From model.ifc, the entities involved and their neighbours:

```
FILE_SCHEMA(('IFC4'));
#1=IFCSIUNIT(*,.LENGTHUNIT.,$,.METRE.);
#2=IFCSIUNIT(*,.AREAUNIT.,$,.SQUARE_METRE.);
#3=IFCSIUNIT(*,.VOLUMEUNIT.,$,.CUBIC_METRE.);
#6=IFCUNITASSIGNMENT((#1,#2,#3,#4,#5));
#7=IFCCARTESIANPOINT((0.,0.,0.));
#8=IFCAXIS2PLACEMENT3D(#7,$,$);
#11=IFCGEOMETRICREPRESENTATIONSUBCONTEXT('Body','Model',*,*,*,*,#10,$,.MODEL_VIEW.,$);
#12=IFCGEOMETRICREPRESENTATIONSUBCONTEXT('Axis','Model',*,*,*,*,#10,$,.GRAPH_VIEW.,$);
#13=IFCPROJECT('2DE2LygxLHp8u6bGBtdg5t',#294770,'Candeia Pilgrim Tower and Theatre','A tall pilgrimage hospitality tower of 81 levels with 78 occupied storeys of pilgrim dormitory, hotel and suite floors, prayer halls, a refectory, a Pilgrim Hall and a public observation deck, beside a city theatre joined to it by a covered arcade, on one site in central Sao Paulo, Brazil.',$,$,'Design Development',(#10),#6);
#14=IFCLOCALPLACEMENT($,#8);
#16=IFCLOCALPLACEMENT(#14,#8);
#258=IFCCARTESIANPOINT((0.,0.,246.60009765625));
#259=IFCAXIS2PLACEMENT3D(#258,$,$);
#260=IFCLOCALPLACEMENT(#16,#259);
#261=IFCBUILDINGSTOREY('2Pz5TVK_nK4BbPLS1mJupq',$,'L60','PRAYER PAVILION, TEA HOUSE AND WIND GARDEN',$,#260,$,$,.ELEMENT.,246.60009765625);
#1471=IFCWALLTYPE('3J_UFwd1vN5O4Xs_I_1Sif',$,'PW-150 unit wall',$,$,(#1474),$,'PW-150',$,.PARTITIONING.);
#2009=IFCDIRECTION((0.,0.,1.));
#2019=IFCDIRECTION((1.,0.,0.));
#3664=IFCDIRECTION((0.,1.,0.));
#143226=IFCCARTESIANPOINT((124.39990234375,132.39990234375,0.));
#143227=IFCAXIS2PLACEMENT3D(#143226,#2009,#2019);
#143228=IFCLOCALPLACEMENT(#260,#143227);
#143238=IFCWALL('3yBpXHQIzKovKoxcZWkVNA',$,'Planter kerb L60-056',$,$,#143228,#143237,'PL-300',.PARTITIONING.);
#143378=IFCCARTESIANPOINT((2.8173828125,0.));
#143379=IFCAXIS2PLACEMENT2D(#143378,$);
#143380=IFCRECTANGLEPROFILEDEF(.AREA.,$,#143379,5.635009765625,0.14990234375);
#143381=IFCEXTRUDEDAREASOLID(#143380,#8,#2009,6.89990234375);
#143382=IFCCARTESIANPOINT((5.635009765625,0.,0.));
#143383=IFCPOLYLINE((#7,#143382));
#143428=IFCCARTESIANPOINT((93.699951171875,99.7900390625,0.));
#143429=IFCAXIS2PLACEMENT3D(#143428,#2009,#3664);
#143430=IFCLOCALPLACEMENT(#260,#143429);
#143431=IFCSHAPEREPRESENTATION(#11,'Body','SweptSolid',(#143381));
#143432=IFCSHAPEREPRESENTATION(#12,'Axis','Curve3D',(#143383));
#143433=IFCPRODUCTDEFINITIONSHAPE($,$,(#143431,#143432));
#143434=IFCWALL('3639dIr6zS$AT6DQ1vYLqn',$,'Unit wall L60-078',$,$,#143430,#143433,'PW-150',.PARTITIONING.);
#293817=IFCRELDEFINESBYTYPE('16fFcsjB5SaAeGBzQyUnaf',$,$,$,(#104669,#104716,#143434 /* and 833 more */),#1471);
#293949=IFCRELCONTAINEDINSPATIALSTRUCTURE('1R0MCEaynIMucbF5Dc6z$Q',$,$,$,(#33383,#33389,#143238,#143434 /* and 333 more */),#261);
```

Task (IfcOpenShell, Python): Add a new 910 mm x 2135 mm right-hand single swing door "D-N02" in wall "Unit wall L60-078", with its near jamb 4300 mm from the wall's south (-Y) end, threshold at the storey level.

```python
import numpy as np
import ifcopenshell
import ifcopenshell.api.feature
import ifcopenshell.api.geometry
import ifcopenshell.api.root
import ifcopenshell.api.spatial
import ifcopenshell.geom
import ifcopenshell.util.element
import ifcopenshell.util.placement
import ifcopenshell.util.representation
import ifcopenshell.util.shape
import ifcopenshell.util.unit

model = ifcopenshell.open("model.ifc")
unit_scale = ifcopenshell.util.unit.calculate_unit_scale(model)
settings = ifcopenshell.geom.settings()


def volume(element):
    """Net volume in cubic metres, openings subtracted."""
    shape = ifcopenshell.geom.create_shape(settings, element)
    return ifcopenshell.util.shape.get_volume(shape.geometry)


wall = model.by_guid("3639dIr6zS$AT6DQ1vYLqn")
storey = ifcopenshell.util.element.get_container(wall, ifc_class="IfcBuildingStorey")
context = ifcopenshell.util.representation.get_context(model, "Model", "Body", "MODEL_VIEW")
before = volume(wall)

width, height, from_end, sill = 0.91, 2.135, 4.3, 0.0  # metres

# The wall runs along its own X axis, and the end named is its -X end.
wall_shape = ifcopenshell.geom.create_shape(settings, wall)
x, y, z = ifcopenshell.util.shape.get_vertices(wall_shape.geometry).T
start = x.min() + from_end
face, thickness = float(y.min()), float(y.max() - y.min())
wall_matrix = ifcopenshell.util.placement.get_local_placement(wall.ObjectPlacement)
level = ifcopenshell.util.placement.get_local_placement(storey.ObjectPlacement)[2, 3]


def in_wall(x, y):
    """Placement at x, y metres in the wall's axes, at sill height."""
    matrix = wall_matrix.copy()
    matrix[:, 3] = wall_matrix @ np.array([x / unit_scale, y / unit_scale, 0.0, 1.0])
    matrix[2, 3] = level + sill / unit_scale
    return matrix


# Opening: a box that overshoots both wall faces by 50 mm.
opening = ifcopenshell.api.root.create_entity(model, ifc_class="IfcOpeningElement", predefined_type="OPENING")
box = ifcopenshell.api.geometry.add_wall_representation(
    model, context=context, length=width, height=height, thickness=thickness + 0.1
)
ifcopenshell.api.geometry.assign_representation(model, product=opening, representation=box)
ifcopenshell.api.geometry.edit_object_placement(model, product=opening, matrix=in_wall(start, face - 0.05), is_si=False)
ifcopenshell.api.feature.add_feature(model, feature=opening, element=wall)

door = ifcopenshell.api.root.create_entity(model, ifc_class="IfcDoor", name="D-N02", predefined_type="DOOR")
door.OverallWidth, door.OverallHeight = width / unit_scale, height / unit_scale
door.OperationType = "SINGLE_SWING_RIGHT"
body = ifcopenshell.api.geometry.add_door_representation(
    model,
    context=context,
    overall_width=door.OverallWidth,
    overall_height=door.OverallHeight,
    operation_type="SINGLE_SWING_RIGHT",
    lining_properties={"LiningDepth": thickness / unit_scale, "ThresholdDepth": thickness / unit_scale},
)
ifcopenshell.api.geometry.assign_representation(model, product=door, representation=body)
ifcopenshell.api.spatial.assign_container(model, products=[door], relating_structure=storey)
ifcopenshell.api.feature.add_filling(model, opening=opening, element=door)

# The lining spans the wall, so the door starts at the wall face.
ifcopenshell.api.geometry.edit_object_placement(model, product=door, matrix=in_wall(start, face), is_si=False)

after = volume(wall)

print(f"wall volume {before:.3f} -> {after:.3f} m3")

model.write("model_rev.ifc")
```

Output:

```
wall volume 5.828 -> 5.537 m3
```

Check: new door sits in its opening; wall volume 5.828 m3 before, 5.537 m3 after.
